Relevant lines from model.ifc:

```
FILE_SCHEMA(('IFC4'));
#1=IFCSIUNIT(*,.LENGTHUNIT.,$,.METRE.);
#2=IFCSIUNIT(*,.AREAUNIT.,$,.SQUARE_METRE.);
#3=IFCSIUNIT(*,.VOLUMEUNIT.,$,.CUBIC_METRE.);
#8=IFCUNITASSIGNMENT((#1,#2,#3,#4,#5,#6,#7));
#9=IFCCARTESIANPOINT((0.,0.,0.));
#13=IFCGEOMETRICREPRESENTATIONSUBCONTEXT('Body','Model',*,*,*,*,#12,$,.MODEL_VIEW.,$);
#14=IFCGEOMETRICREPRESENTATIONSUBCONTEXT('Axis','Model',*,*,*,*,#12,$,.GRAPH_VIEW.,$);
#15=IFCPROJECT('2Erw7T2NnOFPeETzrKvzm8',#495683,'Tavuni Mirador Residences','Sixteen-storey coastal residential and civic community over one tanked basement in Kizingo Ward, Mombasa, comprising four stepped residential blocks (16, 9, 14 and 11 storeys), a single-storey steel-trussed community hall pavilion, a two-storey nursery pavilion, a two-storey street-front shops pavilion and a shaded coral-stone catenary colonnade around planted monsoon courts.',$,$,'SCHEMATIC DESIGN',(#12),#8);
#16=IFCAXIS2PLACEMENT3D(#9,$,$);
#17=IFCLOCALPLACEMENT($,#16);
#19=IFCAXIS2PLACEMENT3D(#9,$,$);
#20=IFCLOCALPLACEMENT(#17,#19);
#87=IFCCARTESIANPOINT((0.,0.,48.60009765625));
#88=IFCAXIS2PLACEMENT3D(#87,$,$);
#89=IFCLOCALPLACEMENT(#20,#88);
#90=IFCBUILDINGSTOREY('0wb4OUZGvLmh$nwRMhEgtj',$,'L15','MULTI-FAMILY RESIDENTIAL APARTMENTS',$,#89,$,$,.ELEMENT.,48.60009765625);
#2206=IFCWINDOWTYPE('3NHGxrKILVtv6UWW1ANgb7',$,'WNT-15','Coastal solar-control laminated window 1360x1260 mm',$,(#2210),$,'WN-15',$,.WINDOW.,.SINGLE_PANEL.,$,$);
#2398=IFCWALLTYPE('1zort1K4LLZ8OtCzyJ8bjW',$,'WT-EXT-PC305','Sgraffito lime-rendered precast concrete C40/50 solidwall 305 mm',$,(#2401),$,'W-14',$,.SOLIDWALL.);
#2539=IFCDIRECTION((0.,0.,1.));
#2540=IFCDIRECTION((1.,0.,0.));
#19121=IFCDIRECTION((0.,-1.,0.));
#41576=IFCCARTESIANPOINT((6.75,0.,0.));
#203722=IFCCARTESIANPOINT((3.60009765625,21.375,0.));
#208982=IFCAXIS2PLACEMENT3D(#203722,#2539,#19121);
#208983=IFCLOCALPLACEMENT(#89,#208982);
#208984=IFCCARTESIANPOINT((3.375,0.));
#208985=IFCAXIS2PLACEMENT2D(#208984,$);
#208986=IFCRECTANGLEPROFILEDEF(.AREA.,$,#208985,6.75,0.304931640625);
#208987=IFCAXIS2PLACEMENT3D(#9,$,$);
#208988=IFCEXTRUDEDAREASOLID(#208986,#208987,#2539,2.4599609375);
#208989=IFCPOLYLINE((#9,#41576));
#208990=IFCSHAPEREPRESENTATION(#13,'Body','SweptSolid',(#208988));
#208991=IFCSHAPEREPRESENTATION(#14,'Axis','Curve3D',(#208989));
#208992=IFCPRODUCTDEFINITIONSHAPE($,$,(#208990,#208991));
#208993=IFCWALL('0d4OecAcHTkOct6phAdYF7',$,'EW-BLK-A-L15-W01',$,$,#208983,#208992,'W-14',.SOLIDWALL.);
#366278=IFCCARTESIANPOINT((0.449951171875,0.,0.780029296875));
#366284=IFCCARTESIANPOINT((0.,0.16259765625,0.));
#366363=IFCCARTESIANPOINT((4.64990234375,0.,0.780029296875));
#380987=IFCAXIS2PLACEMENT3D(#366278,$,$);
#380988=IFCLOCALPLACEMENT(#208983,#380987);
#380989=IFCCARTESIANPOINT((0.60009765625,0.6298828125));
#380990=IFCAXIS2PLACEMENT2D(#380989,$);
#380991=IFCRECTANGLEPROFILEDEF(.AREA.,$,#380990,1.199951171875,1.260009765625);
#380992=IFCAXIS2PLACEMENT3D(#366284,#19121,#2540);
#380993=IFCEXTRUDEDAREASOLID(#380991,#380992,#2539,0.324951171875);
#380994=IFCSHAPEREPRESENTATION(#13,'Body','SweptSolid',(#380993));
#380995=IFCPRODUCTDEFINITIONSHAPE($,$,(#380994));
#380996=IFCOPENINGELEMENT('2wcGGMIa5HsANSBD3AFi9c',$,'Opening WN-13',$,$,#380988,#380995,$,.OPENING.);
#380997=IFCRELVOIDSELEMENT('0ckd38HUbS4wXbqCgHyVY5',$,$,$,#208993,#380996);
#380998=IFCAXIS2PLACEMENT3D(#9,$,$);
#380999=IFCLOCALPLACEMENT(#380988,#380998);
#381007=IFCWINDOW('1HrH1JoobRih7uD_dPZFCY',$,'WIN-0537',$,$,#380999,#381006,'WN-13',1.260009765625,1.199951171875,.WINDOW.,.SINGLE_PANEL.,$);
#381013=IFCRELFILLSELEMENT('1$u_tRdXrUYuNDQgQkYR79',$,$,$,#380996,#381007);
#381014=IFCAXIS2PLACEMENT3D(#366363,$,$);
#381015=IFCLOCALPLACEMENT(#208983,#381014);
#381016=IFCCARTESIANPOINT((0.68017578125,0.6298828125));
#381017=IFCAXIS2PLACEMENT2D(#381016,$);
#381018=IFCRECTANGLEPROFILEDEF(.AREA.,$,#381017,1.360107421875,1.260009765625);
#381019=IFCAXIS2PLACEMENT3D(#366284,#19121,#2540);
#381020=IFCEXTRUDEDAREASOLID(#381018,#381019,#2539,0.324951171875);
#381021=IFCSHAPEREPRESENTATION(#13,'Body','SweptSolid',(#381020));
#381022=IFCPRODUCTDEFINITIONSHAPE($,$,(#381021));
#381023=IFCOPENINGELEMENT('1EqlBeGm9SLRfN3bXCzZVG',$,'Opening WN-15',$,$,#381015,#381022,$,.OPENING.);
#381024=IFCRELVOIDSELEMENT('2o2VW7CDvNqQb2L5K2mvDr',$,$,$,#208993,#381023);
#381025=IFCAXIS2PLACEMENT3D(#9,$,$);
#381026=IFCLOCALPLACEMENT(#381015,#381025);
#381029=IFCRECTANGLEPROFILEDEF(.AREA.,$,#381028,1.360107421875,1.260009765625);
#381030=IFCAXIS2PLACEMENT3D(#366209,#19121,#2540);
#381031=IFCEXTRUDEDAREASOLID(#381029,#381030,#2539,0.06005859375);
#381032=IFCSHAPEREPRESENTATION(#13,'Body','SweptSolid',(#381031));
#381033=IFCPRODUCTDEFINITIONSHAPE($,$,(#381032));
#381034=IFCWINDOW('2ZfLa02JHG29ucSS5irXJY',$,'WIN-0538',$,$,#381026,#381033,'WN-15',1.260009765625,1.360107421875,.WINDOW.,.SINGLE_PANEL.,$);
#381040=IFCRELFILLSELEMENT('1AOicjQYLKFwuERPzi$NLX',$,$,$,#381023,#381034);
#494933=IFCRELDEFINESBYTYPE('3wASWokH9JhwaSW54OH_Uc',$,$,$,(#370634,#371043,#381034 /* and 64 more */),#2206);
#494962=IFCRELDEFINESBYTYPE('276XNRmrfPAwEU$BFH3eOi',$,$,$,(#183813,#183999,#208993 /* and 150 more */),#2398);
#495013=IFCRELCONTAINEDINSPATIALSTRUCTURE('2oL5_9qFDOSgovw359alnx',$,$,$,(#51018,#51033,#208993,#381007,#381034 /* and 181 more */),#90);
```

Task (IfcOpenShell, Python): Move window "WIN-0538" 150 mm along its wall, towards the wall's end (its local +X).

```python
import ifcopenshell
import ifcopenshell.api.geometry
import ifcopenshell.util.placement
import ifcopenshell.util.unit

model = ifcopenshell.open("model.ifc")
unit_scale = ifcopenshell.util.unit.calculate_unit_scale(model)

window = model.by_guid("2ZfLa02JHG29ucSS5irXJY")
opening = window.FillsVoids[0].RelatingOpeningElement
wall = opening.VoidsElements[0].RelatingBuildingElement

wall_matrix = ifcopenshell.util.placement.get_local_placement(wall.ObjectPlacement)
shift = wall_matrix[:3, 0] * 0.15 / unit_scale
before = ifcopenshell.util.placement.get_local_placement(window.ObjectPlacement)[:3, 3].copy()

# The window is placed relative to its opening, so it follows when the opening moves.
matrix = ifcopenshell.util.placement.get_local_placement(opening.ObjectPlacement)
matrix[:3, 3] += shift
ifcopenshell.api.geometry.edit_object_placement(
    model, product=opening, matrix=matrix, is_si=False, should_transform_children=True
)

after = ifcopenshell.util.placement.get_local_placement(window.ObjectPlacement)[:3, 3]
print("window moved by", (after - before).round(3) + 0.0)

model.write("model_edited.ifc")
```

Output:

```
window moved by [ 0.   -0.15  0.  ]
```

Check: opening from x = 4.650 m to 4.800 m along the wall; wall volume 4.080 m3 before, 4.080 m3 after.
